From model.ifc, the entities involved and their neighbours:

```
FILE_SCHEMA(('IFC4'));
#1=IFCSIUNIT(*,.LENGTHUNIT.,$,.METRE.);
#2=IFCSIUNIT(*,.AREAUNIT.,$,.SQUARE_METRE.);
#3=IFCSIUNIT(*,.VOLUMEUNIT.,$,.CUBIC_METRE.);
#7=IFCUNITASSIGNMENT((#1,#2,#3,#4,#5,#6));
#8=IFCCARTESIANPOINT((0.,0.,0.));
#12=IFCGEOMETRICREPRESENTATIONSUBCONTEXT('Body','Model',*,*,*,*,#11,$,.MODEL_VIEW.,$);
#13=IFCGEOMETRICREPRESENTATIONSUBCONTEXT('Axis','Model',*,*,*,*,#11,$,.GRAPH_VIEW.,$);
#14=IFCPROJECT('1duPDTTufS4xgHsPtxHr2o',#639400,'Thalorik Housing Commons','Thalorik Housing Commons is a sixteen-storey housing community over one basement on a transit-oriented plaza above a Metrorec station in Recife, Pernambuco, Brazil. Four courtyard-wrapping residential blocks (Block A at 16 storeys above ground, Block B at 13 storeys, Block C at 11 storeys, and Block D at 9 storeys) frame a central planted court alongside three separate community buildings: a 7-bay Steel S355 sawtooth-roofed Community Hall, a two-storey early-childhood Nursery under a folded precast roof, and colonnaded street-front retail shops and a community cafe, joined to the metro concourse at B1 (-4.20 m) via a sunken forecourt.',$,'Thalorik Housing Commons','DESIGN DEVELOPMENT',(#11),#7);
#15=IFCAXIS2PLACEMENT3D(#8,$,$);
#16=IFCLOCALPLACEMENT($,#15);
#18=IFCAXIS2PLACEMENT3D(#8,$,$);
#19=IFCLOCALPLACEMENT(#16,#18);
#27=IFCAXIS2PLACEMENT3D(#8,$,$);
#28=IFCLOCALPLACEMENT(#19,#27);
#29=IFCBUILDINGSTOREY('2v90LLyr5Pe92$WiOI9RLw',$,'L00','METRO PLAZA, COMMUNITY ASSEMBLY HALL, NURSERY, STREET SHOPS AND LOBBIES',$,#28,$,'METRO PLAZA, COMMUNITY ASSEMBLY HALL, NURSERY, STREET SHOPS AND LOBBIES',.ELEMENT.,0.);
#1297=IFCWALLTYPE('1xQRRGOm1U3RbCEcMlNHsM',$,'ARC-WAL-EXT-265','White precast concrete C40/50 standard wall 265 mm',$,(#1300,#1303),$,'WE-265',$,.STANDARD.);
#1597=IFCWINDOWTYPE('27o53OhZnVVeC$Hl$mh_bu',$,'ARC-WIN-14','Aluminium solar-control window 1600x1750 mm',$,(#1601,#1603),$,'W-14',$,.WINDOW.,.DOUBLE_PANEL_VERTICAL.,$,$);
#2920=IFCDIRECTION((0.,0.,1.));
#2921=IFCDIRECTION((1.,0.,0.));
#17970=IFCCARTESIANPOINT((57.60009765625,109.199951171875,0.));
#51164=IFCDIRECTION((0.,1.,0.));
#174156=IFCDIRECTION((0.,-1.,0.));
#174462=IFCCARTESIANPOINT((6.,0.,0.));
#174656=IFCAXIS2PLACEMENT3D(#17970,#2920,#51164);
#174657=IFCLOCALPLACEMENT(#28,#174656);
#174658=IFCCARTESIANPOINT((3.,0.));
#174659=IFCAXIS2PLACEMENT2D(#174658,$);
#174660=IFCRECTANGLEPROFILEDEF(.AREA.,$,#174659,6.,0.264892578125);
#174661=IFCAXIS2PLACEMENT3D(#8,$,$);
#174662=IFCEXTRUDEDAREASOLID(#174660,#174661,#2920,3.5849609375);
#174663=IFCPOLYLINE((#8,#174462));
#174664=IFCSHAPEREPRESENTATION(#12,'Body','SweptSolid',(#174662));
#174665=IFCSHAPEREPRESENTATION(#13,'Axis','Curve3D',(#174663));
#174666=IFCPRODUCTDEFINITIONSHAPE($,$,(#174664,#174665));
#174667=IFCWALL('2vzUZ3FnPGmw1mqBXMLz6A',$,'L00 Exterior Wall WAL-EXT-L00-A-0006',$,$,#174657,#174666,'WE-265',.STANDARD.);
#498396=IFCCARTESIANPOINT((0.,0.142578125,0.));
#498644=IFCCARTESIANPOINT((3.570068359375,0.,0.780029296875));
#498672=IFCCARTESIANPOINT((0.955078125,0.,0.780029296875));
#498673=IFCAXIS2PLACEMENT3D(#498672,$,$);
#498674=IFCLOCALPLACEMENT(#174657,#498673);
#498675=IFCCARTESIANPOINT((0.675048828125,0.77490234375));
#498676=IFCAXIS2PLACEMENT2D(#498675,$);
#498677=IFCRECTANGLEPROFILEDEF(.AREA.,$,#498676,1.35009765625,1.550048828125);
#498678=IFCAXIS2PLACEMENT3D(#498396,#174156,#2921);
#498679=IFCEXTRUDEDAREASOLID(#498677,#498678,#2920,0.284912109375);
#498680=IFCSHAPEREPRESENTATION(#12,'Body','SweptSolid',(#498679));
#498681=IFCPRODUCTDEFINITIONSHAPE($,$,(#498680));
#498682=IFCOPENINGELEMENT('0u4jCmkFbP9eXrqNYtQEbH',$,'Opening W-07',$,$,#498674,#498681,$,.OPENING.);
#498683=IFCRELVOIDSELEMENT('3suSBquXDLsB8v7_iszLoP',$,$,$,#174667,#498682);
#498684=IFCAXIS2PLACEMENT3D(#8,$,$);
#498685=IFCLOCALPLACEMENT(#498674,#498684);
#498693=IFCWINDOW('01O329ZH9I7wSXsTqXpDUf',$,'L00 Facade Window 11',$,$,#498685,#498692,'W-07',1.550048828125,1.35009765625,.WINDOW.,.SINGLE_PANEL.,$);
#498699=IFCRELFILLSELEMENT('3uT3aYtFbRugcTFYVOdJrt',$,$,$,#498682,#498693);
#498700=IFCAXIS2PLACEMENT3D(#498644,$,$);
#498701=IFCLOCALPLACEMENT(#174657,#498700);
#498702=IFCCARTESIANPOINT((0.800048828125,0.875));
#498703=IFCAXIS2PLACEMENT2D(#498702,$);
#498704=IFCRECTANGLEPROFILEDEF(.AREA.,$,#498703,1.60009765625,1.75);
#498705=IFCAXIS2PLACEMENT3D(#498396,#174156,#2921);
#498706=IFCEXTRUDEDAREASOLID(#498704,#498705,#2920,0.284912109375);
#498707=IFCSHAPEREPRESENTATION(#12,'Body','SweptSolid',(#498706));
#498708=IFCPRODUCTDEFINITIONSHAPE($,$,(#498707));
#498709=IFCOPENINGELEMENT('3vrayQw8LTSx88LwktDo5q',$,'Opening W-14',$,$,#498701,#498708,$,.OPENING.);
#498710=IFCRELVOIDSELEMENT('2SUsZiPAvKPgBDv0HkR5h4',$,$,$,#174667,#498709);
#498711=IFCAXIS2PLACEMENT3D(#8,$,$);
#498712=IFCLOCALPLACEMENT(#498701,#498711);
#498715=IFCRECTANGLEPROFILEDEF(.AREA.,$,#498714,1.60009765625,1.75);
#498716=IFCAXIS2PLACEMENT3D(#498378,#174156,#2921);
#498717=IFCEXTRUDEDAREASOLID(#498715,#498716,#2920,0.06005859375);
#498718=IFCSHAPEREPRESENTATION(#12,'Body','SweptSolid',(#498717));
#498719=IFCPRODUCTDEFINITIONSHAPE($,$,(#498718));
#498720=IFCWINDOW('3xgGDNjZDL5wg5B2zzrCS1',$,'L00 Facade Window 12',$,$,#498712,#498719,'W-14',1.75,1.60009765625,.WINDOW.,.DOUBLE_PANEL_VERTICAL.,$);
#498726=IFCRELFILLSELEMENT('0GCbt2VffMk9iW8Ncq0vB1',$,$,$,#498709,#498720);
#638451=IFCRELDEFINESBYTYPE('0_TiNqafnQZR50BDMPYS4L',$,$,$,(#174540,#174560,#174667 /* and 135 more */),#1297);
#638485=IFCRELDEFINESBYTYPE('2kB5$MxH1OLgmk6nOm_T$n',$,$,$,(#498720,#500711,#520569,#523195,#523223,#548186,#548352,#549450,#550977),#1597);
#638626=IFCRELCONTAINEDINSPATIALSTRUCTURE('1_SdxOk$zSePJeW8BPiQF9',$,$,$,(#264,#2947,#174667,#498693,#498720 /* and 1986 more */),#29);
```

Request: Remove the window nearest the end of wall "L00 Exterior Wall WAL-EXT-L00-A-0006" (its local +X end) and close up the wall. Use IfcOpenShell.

```python
import ifcopenshell
import ifcopenshell.api.feature
import ifcopenshell.api.root
import ifcopenshell.geom
import ifcopenshell.util.shape

model = ifcopenshell.open("model.ifc")
settings = ifcopenshell.geom.settings()


def volume(element):
    """Net volume in cubic metres, openings subtracted."""
    shape = ifcopenshell.geom.create_shape(settings, element)
    return ifcopenshell.util.shape.get_volume(shape.geometry)


window = model.by_id(498720)
opening = window.FillsVoids[0].RelatingOpeningElement
wall = opening.VoidsElements[0].RelatingBuildingElement
before = volume(wall)

ifcopenshell.api.root.remove_product(model, product=window)
ifcopenshell.api.feature.remove_feature(model, feature=opening)

after = volume(wall)

print(f"wall volume {before:.3f} -> {after:.3f} m3")

model.write("model_v2.ifc")
```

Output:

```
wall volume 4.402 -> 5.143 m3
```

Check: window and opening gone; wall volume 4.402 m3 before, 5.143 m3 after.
